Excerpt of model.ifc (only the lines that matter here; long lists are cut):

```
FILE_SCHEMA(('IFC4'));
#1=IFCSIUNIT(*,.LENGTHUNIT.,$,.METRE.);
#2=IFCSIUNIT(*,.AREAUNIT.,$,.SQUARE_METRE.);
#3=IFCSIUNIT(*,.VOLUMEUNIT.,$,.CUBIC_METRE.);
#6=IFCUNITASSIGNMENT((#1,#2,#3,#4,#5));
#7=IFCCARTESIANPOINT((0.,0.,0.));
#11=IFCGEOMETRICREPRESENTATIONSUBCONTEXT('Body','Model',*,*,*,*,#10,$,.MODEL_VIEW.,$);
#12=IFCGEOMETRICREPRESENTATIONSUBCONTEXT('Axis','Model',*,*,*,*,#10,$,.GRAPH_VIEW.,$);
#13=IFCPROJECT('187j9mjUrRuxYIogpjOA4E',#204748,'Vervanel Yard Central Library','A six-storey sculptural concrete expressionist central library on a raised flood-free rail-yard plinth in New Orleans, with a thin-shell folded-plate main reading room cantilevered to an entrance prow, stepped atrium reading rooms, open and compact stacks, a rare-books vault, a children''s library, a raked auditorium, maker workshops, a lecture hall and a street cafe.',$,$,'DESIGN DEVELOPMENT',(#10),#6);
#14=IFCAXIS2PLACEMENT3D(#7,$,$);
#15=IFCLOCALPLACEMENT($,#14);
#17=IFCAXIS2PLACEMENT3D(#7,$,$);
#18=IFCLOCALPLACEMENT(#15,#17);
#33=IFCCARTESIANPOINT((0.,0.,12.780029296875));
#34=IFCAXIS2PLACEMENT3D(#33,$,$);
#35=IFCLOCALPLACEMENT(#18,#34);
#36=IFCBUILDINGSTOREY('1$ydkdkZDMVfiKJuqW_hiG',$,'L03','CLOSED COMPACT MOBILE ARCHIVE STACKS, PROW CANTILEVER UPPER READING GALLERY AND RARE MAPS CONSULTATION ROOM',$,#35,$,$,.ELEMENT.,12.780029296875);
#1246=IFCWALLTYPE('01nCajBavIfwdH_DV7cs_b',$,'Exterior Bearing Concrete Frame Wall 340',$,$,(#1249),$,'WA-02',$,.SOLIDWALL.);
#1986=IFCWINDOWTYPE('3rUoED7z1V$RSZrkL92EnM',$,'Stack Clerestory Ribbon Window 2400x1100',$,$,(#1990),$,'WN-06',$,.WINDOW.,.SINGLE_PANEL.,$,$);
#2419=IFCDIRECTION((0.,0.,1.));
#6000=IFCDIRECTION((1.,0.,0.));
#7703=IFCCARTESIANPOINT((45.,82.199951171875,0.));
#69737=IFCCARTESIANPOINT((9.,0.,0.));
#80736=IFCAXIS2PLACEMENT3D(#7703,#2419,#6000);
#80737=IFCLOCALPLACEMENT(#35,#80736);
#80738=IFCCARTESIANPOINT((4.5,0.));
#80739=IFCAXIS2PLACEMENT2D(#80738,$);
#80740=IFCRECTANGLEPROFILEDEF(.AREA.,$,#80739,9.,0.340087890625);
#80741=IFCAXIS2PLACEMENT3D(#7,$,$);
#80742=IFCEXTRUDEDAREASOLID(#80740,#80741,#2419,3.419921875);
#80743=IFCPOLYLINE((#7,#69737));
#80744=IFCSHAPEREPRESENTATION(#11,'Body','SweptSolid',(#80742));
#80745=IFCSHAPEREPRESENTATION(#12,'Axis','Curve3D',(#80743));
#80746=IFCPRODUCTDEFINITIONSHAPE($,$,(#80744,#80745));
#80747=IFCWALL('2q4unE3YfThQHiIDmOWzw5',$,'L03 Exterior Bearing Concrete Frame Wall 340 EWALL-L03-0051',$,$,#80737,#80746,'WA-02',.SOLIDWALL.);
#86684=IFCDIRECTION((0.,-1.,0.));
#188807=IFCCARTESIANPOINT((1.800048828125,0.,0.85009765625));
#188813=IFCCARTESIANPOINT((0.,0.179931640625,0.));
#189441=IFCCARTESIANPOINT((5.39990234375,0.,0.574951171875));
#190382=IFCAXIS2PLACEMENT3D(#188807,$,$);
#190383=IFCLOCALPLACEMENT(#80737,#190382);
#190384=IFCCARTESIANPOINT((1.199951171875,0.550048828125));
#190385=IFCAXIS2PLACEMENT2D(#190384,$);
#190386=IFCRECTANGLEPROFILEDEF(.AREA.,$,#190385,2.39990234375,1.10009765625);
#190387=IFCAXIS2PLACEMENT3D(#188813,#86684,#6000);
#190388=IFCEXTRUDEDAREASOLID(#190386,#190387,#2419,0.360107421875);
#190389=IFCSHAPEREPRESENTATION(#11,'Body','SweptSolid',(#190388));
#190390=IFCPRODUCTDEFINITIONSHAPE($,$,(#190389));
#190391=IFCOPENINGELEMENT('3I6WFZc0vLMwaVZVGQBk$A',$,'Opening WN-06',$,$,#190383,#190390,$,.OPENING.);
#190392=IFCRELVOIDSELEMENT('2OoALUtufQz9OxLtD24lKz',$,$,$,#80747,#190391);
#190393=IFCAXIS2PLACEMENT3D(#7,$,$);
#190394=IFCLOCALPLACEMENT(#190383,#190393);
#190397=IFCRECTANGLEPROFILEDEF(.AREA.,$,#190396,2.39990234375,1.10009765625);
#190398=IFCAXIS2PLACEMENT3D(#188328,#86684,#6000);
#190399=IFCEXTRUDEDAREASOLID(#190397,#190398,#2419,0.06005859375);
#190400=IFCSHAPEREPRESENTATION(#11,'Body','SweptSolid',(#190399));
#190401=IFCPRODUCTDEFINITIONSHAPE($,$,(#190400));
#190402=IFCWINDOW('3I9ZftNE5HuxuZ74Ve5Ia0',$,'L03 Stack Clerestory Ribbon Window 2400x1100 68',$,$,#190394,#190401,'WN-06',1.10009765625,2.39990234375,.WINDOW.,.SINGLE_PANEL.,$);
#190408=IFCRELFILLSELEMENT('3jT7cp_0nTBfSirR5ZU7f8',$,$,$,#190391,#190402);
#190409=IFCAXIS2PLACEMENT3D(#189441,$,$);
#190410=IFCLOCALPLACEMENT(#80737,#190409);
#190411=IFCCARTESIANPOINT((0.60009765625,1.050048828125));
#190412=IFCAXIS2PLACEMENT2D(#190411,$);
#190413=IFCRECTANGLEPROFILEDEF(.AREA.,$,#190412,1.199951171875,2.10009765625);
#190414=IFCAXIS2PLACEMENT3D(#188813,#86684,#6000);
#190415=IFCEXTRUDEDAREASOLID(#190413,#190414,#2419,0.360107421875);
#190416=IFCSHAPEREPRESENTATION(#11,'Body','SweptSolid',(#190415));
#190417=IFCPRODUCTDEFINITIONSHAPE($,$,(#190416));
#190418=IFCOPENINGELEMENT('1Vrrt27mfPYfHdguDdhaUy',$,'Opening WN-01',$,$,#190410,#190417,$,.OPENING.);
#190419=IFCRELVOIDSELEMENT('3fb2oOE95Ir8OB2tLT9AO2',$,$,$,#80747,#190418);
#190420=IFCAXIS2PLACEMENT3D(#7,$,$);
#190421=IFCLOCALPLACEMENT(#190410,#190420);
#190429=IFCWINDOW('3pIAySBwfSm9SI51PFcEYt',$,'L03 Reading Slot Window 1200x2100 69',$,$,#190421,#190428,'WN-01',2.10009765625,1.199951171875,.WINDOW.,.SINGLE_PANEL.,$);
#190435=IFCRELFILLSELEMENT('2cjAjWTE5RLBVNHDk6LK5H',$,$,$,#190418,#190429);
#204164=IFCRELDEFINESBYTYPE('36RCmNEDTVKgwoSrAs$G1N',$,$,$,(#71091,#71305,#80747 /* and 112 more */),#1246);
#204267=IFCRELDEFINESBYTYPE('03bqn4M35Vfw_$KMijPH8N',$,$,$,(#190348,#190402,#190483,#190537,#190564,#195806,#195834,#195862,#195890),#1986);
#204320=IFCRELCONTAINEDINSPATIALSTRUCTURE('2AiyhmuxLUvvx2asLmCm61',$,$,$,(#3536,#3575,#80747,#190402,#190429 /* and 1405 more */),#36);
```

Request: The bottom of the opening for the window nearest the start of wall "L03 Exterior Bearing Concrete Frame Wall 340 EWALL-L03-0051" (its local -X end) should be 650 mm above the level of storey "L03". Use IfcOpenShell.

```python
import numpy as np
import ifcopenshell
import ifcopenshell.api.geometry
import ifcopenshell.geom
import ifcopenshell.util.element
import ifcopenshell.util.placement
import ifcopenshell.util.shape
import ifcopenshell.util.unit

model = ifcopenshell.open("model.ifc")
unit_scale = ifcopenshell.util.unit.calculate_unit_scale(model)

window = model.by_guid("3I9ZftNE5HuxuZ74Ve5Ia0")
opening = window.FillsVoids[0].RelatingOpeningElement
storey = ifcopenshell.util.element.get_container(window, ifc_class="IfcBuildingStorey")
level = ifcopenshell.util.placement.get_local_placement(storey.ObjectPlacement)[2, 3]

# The opening's origin need not be at the sill, so measure its lowest point.
shape = ifcopenshell.geom.create_shape(ifcopenshell.geom.settings(), opening)
bottom = ifcopenshell.util.shape.get_shape_bottom_elevation(shape, shape.geometry) / unit_scale
dz = level + 0.65 / unit_scale - bottom

shift = np.array([0.0, 0.0, dz])
# The window is placed relative to its opening, so it follows when the opening moves.
matrix = ifcopenshell.util.placement.get_local_placement(opening.ObjectPlacement)
matrix[:3, 3] += shift
ifcopenshell.api.geometry.edit_object_placement(
    model, product=opening, matrix=matrix, is_si=False, should_transform_children=True
)

print(f"moved by {dz * unit_scale:+.3f} m")

model.write("model_v2.ifc")
```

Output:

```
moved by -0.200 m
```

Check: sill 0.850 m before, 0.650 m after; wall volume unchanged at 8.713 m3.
